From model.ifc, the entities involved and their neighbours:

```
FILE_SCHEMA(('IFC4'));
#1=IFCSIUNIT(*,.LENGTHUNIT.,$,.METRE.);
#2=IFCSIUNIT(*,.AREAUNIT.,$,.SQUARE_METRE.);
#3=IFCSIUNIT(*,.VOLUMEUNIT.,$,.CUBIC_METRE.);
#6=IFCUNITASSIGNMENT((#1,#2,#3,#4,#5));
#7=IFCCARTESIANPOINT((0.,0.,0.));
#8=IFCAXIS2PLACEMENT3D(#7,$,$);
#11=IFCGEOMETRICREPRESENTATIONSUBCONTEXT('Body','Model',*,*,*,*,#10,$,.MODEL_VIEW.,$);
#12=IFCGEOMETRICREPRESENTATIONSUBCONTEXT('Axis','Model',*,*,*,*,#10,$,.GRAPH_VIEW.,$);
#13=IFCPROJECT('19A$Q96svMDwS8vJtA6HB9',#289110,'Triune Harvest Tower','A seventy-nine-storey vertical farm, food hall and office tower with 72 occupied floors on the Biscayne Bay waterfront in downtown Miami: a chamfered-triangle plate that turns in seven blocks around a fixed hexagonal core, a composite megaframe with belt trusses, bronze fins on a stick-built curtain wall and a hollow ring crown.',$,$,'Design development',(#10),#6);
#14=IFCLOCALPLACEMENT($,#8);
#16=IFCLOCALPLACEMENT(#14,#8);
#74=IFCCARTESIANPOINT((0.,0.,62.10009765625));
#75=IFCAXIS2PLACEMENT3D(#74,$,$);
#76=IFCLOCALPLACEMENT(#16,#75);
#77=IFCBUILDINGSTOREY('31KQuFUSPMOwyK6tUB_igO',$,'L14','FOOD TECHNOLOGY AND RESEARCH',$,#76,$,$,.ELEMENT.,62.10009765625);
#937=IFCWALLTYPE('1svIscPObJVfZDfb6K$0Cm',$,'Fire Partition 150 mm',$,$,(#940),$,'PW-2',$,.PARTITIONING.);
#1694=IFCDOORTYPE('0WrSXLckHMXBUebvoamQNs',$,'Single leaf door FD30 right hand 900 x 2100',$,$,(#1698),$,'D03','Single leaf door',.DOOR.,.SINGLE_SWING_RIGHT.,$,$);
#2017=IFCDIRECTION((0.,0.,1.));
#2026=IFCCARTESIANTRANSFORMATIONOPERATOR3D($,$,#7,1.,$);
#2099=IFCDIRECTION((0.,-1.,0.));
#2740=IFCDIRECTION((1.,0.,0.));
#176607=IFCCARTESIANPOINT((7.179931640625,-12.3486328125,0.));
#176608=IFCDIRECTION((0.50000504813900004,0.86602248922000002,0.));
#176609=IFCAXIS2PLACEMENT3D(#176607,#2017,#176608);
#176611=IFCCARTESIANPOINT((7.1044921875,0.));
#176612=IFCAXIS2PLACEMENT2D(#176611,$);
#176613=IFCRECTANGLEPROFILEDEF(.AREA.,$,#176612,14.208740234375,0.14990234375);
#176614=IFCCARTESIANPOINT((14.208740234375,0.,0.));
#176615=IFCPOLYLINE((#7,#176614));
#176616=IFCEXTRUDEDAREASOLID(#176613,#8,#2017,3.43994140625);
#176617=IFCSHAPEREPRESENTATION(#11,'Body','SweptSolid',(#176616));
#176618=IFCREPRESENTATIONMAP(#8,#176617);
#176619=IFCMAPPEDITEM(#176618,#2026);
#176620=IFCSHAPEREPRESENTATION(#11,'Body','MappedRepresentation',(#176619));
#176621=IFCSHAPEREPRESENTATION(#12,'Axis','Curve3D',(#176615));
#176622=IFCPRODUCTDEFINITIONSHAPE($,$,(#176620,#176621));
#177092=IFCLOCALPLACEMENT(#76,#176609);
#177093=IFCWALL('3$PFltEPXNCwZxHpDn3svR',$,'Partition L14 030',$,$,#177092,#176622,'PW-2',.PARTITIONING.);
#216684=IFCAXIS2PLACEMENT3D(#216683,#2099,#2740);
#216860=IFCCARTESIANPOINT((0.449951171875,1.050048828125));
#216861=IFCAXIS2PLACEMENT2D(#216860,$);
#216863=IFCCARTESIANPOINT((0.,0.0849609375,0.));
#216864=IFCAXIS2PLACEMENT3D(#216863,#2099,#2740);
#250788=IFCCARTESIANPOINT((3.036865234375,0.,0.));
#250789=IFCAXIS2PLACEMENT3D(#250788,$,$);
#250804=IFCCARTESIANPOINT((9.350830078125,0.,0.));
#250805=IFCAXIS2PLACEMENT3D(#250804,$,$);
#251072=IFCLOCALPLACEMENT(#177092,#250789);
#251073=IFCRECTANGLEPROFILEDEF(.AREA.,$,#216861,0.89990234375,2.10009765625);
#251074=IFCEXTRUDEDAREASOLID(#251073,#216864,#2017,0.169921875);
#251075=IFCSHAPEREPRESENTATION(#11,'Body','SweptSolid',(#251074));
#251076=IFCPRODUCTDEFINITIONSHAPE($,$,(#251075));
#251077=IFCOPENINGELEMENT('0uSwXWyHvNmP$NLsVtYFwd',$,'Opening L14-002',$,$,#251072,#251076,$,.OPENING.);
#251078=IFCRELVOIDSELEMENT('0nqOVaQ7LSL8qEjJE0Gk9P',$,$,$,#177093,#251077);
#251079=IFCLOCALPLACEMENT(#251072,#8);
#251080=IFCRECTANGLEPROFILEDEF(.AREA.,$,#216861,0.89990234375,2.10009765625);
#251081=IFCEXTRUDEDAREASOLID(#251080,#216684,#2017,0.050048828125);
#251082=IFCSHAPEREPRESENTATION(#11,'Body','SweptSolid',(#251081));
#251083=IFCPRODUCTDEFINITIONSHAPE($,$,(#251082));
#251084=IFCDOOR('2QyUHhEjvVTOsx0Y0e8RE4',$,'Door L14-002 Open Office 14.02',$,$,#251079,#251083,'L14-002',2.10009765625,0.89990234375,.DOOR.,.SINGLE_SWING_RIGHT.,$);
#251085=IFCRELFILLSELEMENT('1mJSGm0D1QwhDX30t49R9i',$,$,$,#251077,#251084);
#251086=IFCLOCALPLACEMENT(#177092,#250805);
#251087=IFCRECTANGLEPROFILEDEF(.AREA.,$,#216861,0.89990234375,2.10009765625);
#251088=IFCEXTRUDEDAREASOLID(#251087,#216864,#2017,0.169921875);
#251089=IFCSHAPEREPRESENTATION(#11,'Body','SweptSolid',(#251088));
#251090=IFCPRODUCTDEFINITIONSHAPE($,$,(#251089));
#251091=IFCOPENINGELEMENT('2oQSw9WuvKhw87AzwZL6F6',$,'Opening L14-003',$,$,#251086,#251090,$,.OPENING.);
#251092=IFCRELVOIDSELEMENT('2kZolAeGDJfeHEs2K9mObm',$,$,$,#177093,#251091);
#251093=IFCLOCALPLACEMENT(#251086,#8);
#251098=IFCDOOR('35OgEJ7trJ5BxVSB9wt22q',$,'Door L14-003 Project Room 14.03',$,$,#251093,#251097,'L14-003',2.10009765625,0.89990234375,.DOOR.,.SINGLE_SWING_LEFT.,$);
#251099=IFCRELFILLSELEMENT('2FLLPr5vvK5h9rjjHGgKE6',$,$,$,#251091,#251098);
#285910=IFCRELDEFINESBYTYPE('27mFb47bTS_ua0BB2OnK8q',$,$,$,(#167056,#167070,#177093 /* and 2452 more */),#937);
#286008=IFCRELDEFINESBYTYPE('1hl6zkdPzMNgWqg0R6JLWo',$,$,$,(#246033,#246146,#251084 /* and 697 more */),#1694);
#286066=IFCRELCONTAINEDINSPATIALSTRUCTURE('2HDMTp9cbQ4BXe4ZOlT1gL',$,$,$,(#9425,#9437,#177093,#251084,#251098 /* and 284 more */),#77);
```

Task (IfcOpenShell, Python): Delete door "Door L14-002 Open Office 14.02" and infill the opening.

```python
import ifcopenshell
import ifcopenshell.api.feature
import ifcopenshell.api.root
import ifcopenshell.geom
import ifcopenshell.util.shape

model = ifcopenshell.open("model.ifc")
settings = ifcopenshell.geom.settings()


def volume(element):
    """Net volume in cubic metres, openings subtracted."""
    shape = ifcopenshell.geom.create_shape(settings, element)
    return ifcopenshell.util.shape.get_volume(shape.geometry)


door = model.by_guid("2QyUHhEjvVTOsx0Y0e8RE4")
opening = door.FillsVoids[0].RelatingOpeningElement
wall = opening.VoidsElements[0].RelatingBuildingElement
before = volume(wall)

ifcopenshell.api.root.remove_product(model, product=door)
ifcopenshell.api.feature.remove_feature(model, feature=opening)

after = volume(wall)

print(f"wall volume {before:.3f} -> {after:.3f} m3")

model.write("model_edited.ifc")
```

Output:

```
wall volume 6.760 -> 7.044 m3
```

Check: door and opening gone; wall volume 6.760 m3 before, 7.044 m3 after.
